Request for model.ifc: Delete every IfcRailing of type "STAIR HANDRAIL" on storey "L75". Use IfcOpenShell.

First a look at what the model holds.

```python
import ifcopenshell
import ifcopenshell.util.element

model = ifcopenshell.open("model.ifc")
print(model.schema)
storey = next(s for s in model.by_type("IfcBuildingStorey") if s.Name == "L75")
railings = [e for e in ifcopenshell.util.element.get_decomposition(storey) if e.is_a("IfcRailing")]
seen = {}
for e in railings:
    element_type = ifcopenshell.util.element.get_type(e)
    name = element_type.Name if element_type not in (None, e) else None
    seen[name] = seen.get(name, 0) + 1
for name, count in sorted(seen.items(), key=str):
    print(count, "x", name)
```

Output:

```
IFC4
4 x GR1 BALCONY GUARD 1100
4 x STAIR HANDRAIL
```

```python
import ifcopenshell
import ifcopenshell.api.root
import ifcopenshell.util.element

model = ifcopenshell.open("model.ifc")

storey = next(s for s in model.by_type("IfcBuildingStorey") if s.Name == "L75")
railings = [e for e in ifcopenshell.util.element.get_decomposition(storey) if e.is_a("IfcRailing")]
targets = [e for e in railings if (t := ifcopenshell.util.element.get_type(e)) not in (None, e) and t.Name == "STAIR HANDRAIL"]

for e in targets:
    ifcopenshell.api.root.remove_product(model, product=e)
print(len(targets), "removed")

model.write("model_rev.ifc")
```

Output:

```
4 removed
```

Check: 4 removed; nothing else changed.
